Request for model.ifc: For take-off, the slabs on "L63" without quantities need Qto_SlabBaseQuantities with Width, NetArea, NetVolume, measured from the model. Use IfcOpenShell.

First a look at what the model holds.

```python
import ifcopenshell
import ifcopenshell.util.element
import ifcopenshell.util.unit

model = ifcopenshell.open("model.ifc")
print(model.schema)
for unit_type in ("LENGTHUNIT", "AREAUNIT", "VOLUMEUNIT"):
    print(unit_type, ifcopenshell.util.unit.calculate_unit_scale(model, unit_type))
storey = next(s for s in model.by_type("IfcBuildingStorey") if s.Name == "L63")
slabs = [e for e in ifcopenshell.util.element.get_decomposition(storey) if e.is_a("IfcSlab")]
for e in sorted(slabs, key=lambda e: e.id()):
    print(e.id(), e.is_a(), e.Name, list(ifcopenshell.util.element.get_psets(e, qtos_only=True)), sep=" | ")
```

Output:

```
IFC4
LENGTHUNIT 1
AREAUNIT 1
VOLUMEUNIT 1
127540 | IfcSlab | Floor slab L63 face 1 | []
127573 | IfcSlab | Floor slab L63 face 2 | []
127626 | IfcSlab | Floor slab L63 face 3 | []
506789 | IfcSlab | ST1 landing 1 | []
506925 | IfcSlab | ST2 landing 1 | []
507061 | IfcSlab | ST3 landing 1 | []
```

```python
import ifcopenshell
import ifcopenshell.api.pset
import ifcopenshell.geom
import ifcopenshell.util.element
import ifcopenshell.util.shape
import ifcopenshell.util.unit

model = ifcopenshell.open("model.ifc")
unit_scale = ifcopenshell.util.unit.calculate_unit_scale(model)
area_scale = ifcopenshell.util.unit.calculate_unit_scale(model, "AREAUNIT")
volume_scale = ifcopenshell.util.unit.calculate_unit_scale(model, "VOLUMEUNIT")
settings = ifcopenshell.geom.settings()

storey = next(s for s in model.by_type("IfcBuildingStorey") if s.Name == "L63")
slabs = [e for e in ifcopenshell.util.element.get_decomposition(storey) if e.is_a("IfcSlab")]

for e in sorted(slabs, key=lambda e: e.id()):
    if ifcopenshell.util.element.get_psets(e, qtos_only=True, should_inherit=False):
        continue
    # Geometry comes back in metres, in the element's own axes.
    shape = ifcopenshell.geom.create_shape(settings, e)
    values = {
        "Width": ifcopenshell.util.shape.get_z(shape.geometry) / unit_scale,
        "NetArea": ifcopenshell.util.shape.get_footprint_area(shape.geometry) / area_scale,
        "NetVolume": ifcopenshell.util.shape.get_volume(shape.geometry) / volume_scale,
    }
    qto = ifcopenshell.api.pset.add_qto(model, product=e, name="Qto_SlabBaseQuantities")
    ifcopenshell.api.pset.edit_qto(model, qto=qto, properties=values)
    print(e.id(), {k: round(v, 3) for k, v in values.items()})

model.write("model-out.ifc")
```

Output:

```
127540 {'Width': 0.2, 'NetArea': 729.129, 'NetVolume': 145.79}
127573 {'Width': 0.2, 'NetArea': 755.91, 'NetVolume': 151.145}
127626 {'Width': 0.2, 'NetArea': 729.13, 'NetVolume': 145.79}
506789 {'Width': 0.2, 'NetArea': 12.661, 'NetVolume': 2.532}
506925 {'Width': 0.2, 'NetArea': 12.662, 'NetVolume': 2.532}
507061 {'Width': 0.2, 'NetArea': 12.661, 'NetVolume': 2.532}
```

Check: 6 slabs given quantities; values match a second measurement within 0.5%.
